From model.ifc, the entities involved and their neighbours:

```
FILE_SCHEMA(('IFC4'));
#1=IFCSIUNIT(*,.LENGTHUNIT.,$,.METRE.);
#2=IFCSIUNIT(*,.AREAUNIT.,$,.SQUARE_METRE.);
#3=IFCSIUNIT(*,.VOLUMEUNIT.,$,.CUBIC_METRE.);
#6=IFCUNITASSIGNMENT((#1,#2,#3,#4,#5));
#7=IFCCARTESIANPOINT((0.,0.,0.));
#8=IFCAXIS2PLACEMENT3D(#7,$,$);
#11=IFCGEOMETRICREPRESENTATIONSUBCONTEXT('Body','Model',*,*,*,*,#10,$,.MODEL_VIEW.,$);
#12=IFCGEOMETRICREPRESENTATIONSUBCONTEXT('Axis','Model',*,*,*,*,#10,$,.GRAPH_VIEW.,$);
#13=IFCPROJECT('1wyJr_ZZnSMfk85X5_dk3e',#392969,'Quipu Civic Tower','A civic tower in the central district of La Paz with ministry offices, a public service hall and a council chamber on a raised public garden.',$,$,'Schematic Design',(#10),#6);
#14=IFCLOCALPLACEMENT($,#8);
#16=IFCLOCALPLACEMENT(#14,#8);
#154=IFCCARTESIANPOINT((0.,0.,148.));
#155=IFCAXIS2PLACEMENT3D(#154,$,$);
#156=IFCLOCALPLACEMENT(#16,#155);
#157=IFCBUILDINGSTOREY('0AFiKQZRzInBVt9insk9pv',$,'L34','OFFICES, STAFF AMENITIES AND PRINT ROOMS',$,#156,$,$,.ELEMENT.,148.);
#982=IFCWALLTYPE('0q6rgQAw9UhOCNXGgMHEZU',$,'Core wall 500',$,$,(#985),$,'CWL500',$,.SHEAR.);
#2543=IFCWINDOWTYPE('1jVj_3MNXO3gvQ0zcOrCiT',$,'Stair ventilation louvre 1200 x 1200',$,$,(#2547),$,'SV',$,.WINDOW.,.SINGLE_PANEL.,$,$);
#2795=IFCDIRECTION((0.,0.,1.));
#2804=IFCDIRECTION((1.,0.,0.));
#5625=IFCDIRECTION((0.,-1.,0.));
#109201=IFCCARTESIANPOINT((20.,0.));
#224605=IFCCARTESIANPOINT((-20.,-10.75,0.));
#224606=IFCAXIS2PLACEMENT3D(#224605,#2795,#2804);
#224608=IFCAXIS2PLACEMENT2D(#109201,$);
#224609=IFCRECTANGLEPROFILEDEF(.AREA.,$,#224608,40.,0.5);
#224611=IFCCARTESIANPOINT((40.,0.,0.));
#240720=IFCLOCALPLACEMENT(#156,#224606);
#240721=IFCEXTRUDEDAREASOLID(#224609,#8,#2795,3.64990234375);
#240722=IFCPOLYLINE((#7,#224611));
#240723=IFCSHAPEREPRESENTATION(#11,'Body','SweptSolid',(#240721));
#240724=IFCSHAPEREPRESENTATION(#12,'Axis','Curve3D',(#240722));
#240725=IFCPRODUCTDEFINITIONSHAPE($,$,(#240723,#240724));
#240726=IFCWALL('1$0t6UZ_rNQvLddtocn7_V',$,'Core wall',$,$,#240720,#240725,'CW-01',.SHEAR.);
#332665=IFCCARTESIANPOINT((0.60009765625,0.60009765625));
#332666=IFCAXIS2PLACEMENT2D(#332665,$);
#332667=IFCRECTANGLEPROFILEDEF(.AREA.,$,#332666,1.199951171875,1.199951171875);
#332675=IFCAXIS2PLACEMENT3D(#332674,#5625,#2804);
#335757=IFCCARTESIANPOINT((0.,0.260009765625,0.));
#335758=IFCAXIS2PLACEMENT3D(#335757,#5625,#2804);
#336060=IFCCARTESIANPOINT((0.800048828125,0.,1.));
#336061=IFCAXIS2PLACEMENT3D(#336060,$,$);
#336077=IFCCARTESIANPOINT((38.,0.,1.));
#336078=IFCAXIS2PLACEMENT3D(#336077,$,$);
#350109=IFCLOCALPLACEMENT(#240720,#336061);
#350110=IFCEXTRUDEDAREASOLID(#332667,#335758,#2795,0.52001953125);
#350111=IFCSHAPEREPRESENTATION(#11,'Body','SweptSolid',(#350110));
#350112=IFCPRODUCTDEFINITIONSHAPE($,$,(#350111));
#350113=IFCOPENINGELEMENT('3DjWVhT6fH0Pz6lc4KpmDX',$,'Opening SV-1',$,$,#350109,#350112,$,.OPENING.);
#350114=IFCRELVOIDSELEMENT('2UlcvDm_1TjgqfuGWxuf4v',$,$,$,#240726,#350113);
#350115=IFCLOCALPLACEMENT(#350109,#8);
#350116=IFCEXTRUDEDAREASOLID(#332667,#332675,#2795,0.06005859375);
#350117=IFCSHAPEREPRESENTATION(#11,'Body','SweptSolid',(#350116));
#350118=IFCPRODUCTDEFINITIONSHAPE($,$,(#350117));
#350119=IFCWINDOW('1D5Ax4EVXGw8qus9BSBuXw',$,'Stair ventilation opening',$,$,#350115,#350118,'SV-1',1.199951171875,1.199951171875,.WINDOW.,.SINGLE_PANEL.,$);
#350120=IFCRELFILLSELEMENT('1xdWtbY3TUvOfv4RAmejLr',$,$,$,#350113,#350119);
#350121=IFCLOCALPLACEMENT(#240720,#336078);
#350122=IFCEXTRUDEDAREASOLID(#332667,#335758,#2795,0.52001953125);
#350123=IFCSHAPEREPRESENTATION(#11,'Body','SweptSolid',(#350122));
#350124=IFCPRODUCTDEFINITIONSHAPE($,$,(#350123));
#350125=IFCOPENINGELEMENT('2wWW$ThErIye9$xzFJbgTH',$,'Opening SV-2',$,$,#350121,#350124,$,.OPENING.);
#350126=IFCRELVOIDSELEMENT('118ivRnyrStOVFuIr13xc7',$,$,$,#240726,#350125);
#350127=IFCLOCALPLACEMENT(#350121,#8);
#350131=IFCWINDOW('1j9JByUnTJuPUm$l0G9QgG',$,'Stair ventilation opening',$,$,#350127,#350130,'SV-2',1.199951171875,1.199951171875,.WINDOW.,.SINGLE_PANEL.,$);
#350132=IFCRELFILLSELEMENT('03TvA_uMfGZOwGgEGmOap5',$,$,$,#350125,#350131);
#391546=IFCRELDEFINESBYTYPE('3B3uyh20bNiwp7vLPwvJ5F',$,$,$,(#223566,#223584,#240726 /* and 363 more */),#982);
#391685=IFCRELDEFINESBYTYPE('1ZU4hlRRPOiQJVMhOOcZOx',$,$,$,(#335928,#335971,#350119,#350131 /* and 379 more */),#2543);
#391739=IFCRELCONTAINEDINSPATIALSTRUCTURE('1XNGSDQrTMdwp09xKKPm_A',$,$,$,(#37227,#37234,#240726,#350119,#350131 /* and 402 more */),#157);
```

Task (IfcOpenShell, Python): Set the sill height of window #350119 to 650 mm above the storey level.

```python
import numpy as np
import ifcopenshell
import ifcopenshell.api.geometry
import ifcopenshell.geom
import ifcopenshell.util.element
import ifcopenshell.util.placement
import ifcopenshell.util.shape
import ifcopenshell.util.unit

model = ifcopenshell.open("model.ifc")
unit_scale = ifcopenshell.util.unit.calculate_unit_scale(model)

window = model.by_guid("1D5Ax4EVXGw8qus9BSBuXw")
opening = window.FillsVoids[0].RelatingOpeningElement
storey = ifcopenshell.util.element.get_container(window, ifc_class="IfcBuildingStorey")
level = ifcopenshell.util.placement.get_local_placement(storey.ObjectPlacement)[2, 3]

# The opening's origin need not be at the sill, so measure its lowest point.
shape = ifcopenshell.geom.create_shape(ifcopenshell.geom.settings(), opening)
bottom = ifcopenshell.util.shape.get_shape_bottom_elevation(shape, shape.geometry) / unit_scale
dz = level + 0.65 - bottom

shift = np.array([0.0, 0.0, dz])
# The window is placed relative to its opening, so it follows when the opening moves.
matrix = ifcopenshell.util.placement.get_local_placement(opening.ObjectPlacement)
matrix[:3, 3] += shift
ifcopenshell.api.geometry.edit_object_placement(
    model, product=opening, matrix=matrix, is_si=False, should_transform_children=True
)

print(f"moved by {dz * unit_scale:+.3f} m")

model.write("model_edited.ifc")
```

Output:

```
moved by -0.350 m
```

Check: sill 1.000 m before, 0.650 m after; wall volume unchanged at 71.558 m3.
